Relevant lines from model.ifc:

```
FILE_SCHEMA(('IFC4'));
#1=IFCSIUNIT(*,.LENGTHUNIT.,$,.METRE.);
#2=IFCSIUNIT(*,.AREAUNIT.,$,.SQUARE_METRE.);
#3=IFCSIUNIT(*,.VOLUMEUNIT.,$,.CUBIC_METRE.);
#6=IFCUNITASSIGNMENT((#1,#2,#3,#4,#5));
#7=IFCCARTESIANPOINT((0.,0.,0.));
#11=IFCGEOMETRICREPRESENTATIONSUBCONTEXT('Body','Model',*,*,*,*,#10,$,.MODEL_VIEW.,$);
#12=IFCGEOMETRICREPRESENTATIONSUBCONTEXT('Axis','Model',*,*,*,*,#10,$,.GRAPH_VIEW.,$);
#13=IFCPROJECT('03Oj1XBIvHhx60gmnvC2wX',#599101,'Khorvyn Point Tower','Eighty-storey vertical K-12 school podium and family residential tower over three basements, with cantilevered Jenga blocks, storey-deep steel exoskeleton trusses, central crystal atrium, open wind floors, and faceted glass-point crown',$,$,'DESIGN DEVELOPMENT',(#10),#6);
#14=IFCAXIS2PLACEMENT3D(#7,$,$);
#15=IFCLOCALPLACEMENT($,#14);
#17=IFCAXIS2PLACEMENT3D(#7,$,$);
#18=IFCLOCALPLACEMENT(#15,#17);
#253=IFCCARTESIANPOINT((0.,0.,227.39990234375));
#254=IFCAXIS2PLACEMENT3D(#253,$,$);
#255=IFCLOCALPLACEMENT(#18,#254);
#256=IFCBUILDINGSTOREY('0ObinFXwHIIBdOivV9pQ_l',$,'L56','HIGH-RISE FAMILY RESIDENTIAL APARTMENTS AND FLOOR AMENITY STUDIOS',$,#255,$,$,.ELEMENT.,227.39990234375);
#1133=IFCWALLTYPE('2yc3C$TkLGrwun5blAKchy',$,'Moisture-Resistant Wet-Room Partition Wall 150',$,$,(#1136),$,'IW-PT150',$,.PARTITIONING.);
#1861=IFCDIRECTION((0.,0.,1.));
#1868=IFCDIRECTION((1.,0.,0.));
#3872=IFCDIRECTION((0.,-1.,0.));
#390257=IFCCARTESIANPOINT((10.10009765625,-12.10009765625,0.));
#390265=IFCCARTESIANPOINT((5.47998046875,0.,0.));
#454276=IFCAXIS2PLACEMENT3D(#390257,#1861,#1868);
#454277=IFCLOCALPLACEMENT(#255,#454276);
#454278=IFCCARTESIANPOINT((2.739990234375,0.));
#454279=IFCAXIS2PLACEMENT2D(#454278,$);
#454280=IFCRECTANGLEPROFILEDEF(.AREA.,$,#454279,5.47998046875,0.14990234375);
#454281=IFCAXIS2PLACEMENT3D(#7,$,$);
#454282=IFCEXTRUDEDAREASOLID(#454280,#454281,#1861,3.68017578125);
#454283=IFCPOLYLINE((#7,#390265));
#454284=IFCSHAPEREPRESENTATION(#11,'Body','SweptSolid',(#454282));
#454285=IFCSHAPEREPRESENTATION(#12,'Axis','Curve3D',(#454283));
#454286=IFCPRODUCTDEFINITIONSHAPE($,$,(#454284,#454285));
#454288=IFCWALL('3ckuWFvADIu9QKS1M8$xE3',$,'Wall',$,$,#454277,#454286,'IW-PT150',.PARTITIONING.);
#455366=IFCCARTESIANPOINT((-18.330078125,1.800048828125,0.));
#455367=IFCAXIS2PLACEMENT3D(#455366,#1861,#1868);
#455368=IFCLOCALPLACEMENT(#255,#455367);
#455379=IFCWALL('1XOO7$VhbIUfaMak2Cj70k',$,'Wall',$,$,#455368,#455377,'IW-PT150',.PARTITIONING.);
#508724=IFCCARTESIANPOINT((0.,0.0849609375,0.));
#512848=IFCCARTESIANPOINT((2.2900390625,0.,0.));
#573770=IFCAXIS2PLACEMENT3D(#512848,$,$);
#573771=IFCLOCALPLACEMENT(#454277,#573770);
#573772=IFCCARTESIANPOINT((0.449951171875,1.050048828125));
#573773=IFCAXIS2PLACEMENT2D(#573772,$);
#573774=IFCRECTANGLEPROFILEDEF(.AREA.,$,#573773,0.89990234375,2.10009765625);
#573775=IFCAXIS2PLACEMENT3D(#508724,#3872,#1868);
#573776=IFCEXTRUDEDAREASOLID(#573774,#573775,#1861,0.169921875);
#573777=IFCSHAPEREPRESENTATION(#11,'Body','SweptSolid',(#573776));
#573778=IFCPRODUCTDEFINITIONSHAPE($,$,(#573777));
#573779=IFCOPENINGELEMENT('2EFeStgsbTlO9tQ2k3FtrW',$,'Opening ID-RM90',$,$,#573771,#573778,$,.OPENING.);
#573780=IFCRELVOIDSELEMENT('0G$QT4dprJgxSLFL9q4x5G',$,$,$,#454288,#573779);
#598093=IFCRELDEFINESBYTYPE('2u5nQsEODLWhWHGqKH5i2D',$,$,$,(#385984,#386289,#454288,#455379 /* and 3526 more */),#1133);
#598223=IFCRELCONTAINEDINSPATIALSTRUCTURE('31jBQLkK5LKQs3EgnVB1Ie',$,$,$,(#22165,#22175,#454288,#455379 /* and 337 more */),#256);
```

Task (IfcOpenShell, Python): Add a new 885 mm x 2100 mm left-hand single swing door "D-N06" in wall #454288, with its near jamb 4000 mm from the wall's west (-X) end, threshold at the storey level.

```python
import numpy as np
import ifcopenshell
import ifcopenshell.api.feature
import ifcopenshell.api.geometry
import ifcopenshell.api.root
import ifcopenshell.api.spatial
import ifcopenshell.geom
import ifcopenshell.util.element
import ifcopenshell.util.placement
import ifcopenshell.util.representation
import ifcopenshell.util.shape
import ifcopenshell.util.unit

model = ifcopenshell.open("model.ifc")
unit_scale = ifcopenshell.util.unit.calculate_unit_scale(model)
settings = ifcopenshell.geom.settings()


def volume(element):
    """Net volume in cubic metres, openings subtracted."""
    shape = ifcopenshell.geom.create_shape(settings, element)
    return ifcopenshell.util.shape.get_volume(shape.geometry)


wall = model.by_guid("3ckuWFvADIu9QKS1M8$xE3")
storey = ifcopenshell.util.element.get_container(wall, ifc_class="IfcBuildingStorey")
context = ifcopenshell.util.representation.get_context(model, "Model", "Body", "MODEL_VIEW")
before = volume(wall)

width, height, from_end, sill = 0.885, 2.1, 4, 0.0  # metres

# The wall runs along its own X axis, and the end named is its -X end.
wall_shape = ifcopenshell.geom.create_shape(settings, wall)
x, y, z = ifcopenshell.util.shape.get_vertices(wall_shape.geometry).T
start = x.min() + from_end
face, thickness = float(y.min()), float(y.max() - y.min())
wall_matrix = ifcopenshell.util.placement.get_local_placement(wall.ObjectPlacement)
level = ifcopenshell.util.placement.get_local_placement(storey.ObjectPlacement)[2, 3]


def in_wall(x, y):
    """Placement at x, y metres in the wall's axes, at sill height."""
    matrix = wall_matrix.copy()
    matrix[:, 3] = wall_matrix @ np.array([x / unit_scale, y / unit_scale, 0.0, 1.0])
    matrix[2, 3] = level + sill / unit_scale
    return matrix


# Opening: a box that overshoots both wall faces by 50 mm.
opening = ifcopenshell.api.root.create_entity(model, ifc_class="IfcOpeningElement", predefined_type="OPENING")
box = ifcopenshell.api.geometry.add_wall_representation(
    model, context=context, length=width, height=height, thickness=thickness + 0.1
)
ifcopenshell.api.geometry.assign_representation(model, product=opening, representation=box)
ifcopenshell.api.geometry.edit_object_placement(model, product=opening, matrix=in_wall(start, face - 0.05), is_si=False)
ifcopenshell.api.feature.add_feature(model, feature=opening, element=wall)

door = ifcopenshell.api.root.create_entity(model, ifc_class="IfcDoor", name="D-N06", predefined_type="DOOR")
door.OverallWidth, door.OverallHeight = width / unit_scale, height / unit_scale
door.OperationType = "SINGLE_SWING_LEFT"
body = ifcopenshell.api.geometry.add_door_representation(
    model,
    context=context,
    overall_width=door.OverallWidth,
    overall_height=door.OverallHeight,
    operation_type="SINGLE_SWING_LEFT",
    lining_properties={"LiningDepth": thickness / unit_scale, "ThresholdDepth": thickness / unit_scale},
)
ifcopenshell.api.geometry.assign_representation(model, product=door, representation=body)
ifcopenshell.api.spatial.assign_container(model, products=[door], relating_structure=storey)
ifcopenshell.api.feature.add_filling(model, opening=opening, element=door)

# The lining spans the wall, so the door starts at the wall face.
ifcopenshell.api.geometry.edit_object_placement(model, product=door, matrix=in_wall(start, face), is_si=False)

after = volume(wall)

print(f"wall volume {before:.3f} -> {after:.3f} m3")

model.write("model_v2.ifc")
```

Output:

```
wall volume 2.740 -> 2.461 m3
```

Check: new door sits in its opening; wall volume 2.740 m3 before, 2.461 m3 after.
